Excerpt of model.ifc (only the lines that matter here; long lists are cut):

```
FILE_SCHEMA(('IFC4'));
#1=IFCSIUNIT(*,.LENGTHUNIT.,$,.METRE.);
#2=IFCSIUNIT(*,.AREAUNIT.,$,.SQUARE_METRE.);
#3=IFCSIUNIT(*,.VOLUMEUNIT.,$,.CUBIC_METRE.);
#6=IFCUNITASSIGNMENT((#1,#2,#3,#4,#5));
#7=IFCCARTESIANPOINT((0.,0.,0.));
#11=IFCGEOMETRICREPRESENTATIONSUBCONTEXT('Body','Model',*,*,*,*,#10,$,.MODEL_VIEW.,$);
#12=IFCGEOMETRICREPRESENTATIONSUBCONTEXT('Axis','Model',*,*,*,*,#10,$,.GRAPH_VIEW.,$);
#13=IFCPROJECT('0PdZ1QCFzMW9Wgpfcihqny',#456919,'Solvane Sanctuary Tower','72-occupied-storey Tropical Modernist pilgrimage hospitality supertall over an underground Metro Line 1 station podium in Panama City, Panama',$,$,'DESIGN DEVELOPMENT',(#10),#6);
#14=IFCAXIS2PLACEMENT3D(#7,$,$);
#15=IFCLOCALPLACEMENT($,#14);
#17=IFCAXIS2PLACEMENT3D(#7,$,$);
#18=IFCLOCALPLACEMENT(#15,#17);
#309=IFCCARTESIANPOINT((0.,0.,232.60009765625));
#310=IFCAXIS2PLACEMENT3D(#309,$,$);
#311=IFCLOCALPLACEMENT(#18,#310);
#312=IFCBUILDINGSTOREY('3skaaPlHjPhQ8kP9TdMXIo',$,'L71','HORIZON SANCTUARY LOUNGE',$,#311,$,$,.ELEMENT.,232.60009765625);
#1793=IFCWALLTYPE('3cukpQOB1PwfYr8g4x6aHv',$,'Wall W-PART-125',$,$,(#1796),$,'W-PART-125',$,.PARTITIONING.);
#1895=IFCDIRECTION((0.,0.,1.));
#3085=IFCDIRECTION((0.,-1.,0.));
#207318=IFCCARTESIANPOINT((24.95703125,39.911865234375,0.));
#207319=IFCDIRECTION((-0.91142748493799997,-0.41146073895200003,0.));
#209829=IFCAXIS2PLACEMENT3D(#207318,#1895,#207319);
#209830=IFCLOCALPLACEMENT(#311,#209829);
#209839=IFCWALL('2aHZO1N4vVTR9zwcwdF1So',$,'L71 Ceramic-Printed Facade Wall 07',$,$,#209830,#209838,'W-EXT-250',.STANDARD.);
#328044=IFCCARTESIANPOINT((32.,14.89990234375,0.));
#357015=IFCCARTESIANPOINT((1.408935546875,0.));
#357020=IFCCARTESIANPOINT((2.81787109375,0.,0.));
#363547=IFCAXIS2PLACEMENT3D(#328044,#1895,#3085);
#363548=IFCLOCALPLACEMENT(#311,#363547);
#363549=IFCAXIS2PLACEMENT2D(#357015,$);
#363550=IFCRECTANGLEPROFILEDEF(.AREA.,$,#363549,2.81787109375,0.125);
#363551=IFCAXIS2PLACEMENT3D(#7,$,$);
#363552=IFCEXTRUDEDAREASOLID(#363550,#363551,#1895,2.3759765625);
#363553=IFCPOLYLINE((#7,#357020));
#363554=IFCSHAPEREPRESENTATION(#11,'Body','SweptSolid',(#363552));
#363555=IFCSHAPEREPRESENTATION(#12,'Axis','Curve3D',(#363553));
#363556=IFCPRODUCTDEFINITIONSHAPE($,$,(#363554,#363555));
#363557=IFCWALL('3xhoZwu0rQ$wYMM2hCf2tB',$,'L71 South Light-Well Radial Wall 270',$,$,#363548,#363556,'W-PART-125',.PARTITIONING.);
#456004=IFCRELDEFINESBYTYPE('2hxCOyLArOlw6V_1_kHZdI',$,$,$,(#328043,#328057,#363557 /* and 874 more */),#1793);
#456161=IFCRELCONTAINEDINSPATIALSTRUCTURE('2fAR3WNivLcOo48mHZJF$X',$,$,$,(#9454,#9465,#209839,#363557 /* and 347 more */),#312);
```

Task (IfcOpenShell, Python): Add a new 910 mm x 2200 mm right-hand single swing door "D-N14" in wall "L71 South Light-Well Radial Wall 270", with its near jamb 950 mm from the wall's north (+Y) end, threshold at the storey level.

```python
import numpy as np
import ifcopenshell
import ifcopenshell.api.feature
import ifcopenshell.api.geometry
import ifcopenshell.api.root
import ifcopenshell.api.spatial
import ifcopenshell.geom
import ifcopenshell.util.element
import ifcopenshell.util.placement
import ifcopenshell.util.representation
import ifcopenshell.util.shape
import ifcopenshell.util.unit

model = ifcopenshell.open("model.ifc")
unit_scale = ifcopenshell.util.unit.calculate_unit_scale(model)
settings = ifcopenshell.geom.settings()


def volume(element):
    """Net volume in cubic metres, openings subtracted."""
    shape = ifcopenshell.geom.create_shape(settings, element)
    return ifcopenshell.util.shape.get_volume(shape.geometry)


wall = model.by_guid("3xhoZwu0rQ$wYMM2hCf2tB")
storey = ifcopenshell.util.element.get_container(wall, ifc_class="IfcBuildingStorey")
context = ifcopenshell.util.representation.get_context(model, "Model", "Body", "MODEL_VIEW")
before = volume(wall)

width, height, from_end, sill = 0.91, 2.2, 0.95, 0.0  # metres

# The wall runs along its own X axis, and the end named is its -X end.
wall_shape = ifcopenshell.geom.create_shape(settings, wall)
x, y, z = ifcopenshell.util.shape.get_vertices(wall_shape.geometry).T
start = x.min() + from_end
face, thickness = float(y.min()), float(y.max() - y.min())
wall_matrix = ifcopenshell.util.placement.get_local_placement(wall.ObjectPlacement)
level = ifcopenshell.util.placement.get_local_placement(storey.ObjectPlacement)[2, 3]


def in_wall(x, y):
    """Placement at x, y metres in the wall's axes, at sill height."""
    matrix = wall_matrix.copy()
    matrix[:, 3] = wall_matrix @ np.array([x / unit_scale, y / unit_scale, 0.0, 1.0])
    matrix[2, 3] = level + sill / unit_scale
    return matrix


# Opening: a box that overshoots both wall faces by 50 mm.
opening = ifcopenshell.api.root.create_entity(model, ifc_class="IfcOpeningElement", predefined_type="OPENING")
box = ifcopenshell.api.geometry.add_wall_representation(
    model, context=context, length=width, height=height, thickness=thickness + 0.1
)
ifcopenshell.api.geometry.assign_representation(model, product=opening, representation=box)
ifcopenshell.api.geometry.edit_object_placement(model, product=opening, matrix=in_wall(start, face - 0.05), is_si=False)
ifcopenshell.api.feature.add_feature(model, feature=opening, element=wall)

door = ifcopenshell.api.root.create_entity(model, ifc_class="IfcDoor", name="D-N14", predefined_type="DOOR")
door.OverallWidth, door.OverallHeight = width / unit_scale, height / unit_scale
door.OperationType = "SINGLE_SWING_RIGHT"
body = ifcopenshell.api.geometry.add_door_representation(
    model,
    context=context,
    overall_width=door.OverallWidth,
    overall_height=door.OverallHeight,
    operation_type="SINGLE_SWING_RIGHT",
    lining_properties={"LiningDepth": thickness / unit_scale, "ThresholdDepth": thickness / unit_scale},
)
ifcopenshell.api.geometry.assign_representation(model, product=door, representation=body)
ifcopenshell.api.spatial.assign_container(model, products=[door], relating_structure=storey)
ifcopenshell.api.feature.add_filling(model, opening=opening, element=door)

# The lining spans the wall, so the door starts at the wall face.
ifcopenshell.api.geometry.edit_object_placement(model, product=door, matrix=in_wall(start, face), is_si=False)

after = volume(wall)

print(f"wall volume {before:.3f} -> {after:.3f} m3")

model.write("model_edited.ifc")
```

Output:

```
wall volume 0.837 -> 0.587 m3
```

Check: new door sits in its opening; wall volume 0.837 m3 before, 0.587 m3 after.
